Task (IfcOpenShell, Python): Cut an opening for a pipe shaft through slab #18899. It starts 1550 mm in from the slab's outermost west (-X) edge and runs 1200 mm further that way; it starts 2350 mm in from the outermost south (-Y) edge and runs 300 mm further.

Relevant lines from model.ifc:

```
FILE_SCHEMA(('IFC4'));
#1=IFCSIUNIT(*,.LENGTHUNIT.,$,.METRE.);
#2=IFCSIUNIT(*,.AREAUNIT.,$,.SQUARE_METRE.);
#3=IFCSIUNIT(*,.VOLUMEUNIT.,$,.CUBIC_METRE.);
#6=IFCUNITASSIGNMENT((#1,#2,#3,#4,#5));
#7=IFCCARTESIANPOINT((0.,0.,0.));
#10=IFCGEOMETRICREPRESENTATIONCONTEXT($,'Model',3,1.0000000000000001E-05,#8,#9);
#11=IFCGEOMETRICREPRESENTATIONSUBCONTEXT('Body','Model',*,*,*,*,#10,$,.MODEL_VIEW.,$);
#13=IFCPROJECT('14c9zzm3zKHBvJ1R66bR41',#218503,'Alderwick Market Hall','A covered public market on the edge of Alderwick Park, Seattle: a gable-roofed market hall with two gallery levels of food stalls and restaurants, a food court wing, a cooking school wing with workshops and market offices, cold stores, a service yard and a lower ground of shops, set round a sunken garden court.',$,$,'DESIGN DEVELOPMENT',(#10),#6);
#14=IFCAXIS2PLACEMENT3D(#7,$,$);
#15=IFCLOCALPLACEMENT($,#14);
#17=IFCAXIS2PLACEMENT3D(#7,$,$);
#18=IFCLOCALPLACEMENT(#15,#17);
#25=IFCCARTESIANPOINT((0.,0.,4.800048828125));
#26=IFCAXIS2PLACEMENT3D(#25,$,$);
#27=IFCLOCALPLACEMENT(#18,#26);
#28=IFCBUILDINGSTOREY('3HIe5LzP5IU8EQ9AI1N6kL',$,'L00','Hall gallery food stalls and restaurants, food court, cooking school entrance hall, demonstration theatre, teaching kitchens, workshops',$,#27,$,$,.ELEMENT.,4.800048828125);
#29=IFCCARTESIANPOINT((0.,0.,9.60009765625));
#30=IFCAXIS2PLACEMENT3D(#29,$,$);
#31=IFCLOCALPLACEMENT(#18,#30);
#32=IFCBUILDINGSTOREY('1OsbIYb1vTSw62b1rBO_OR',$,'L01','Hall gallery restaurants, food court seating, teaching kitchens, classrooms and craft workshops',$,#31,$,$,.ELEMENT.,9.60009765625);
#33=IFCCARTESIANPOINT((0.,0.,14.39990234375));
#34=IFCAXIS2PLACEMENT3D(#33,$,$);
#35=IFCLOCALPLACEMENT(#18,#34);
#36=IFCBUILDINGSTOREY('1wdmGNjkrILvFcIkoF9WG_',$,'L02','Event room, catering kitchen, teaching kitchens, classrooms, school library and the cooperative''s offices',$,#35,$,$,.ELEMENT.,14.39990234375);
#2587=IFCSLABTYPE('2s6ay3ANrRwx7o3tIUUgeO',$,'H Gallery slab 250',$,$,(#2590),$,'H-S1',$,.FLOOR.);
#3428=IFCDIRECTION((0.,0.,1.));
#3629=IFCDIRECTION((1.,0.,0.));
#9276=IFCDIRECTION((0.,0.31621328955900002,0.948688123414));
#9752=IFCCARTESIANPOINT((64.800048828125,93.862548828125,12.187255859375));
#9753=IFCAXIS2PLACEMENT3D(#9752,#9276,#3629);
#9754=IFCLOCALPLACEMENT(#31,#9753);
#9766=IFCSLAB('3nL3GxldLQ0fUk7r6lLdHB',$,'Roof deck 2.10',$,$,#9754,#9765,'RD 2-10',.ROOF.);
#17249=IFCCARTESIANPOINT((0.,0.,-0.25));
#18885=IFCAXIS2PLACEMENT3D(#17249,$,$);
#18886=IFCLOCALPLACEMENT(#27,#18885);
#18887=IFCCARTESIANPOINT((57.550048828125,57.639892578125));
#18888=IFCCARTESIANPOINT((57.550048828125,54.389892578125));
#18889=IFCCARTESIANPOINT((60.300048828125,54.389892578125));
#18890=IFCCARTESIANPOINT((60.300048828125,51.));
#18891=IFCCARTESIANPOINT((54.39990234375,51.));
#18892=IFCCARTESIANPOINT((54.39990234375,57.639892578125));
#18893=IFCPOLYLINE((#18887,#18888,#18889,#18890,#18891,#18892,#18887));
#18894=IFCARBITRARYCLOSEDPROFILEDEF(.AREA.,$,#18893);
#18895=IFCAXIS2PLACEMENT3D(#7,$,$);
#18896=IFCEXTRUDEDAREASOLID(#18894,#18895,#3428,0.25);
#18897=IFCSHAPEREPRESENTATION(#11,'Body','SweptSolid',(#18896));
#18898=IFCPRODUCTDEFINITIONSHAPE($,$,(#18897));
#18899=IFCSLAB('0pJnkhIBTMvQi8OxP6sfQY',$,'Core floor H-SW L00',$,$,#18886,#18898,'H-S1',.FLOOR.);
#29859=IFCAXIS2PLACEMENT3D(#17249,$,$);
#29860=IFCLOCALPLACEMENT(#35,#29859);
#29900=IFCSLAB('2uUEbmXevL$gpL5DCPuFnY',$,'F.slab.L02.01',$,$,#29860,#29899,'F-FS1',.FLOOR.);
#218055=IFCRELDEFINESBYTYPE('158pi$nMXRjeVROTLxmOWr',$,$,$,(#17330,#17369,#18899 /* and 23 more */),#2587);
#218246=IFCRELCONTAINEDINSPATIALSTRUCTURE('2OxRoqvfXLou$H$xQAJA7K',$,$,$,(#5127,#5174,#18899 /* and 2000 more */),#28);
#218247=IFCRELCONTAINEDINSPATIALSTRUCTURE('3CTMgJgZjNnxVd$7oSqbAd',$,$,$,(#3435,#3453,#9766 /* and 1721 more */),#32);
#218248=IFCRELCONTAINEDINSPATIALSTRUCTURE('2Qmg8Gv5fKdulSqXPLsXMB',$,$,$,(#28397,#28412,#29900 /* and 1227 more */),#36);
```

```python
import numpy as np
import ifcopenshell
import ifcopenshell.api.feature
import ifcopenshell.api.geometry
import ifcopenshell.api.root
import ifcopenshell.geom
import ifcopenshell.util.placement
import ifcopenshell.util.representation
import ifcopenshell.util.shape
import ifcopenshell.util.unit

model = ifcopenshell.open("model.ifc")
unit_scale = ifcopenshell.util.unit.calculate_unit_scale(model)
settings = ifcopenshell.geom.settings()


def volume(element):
    """Net volume in cubic metres, openings subtracted."""
    shape = ifcopenshell.geom.create_shape(settings, element)
    return ifcopenshell.util.shape.get_volume(shape.geometry)


slab = model.by_id(18899)
before = volume(slab)

# Extent in the slab's own axes, in metres. The edges named are its -X and -Y sides.
slab_shape = ifcopenshell.geom.create_shape(settings, slab)
vertices = ifcopenshell.util.shape.get_vertices(slab_shape.geometry)
x_min, y_min, bottom = vertices.min(axis=0)
top = vertices[:, 2].max()

opening = ifcopenshell.api.root.create_entity(model, ifc_class="IfcOpeningElement", name="Pipe shaft opening", predefined_type="OPENING")
context = ifcopenshell.util.representation.get_context(model, "Model", "Body", "MODEL_VIEW")
width, depth = 1.2, 0.3
outline = [(0.0, 0.0), (width, 0.0), (width, depth), (0.0, depth), (0.0, 0.0)]
# Overshoot both faces by 50 mm so the cut is clean.
shape = ifcopenshell.api.geometry.add_slab_representation(
    model, context=context, depth=top - bottom + 0.1, polyline=outline
)
ifcopenshell.api.geometry.assign_representation(model, product=opening, representation=shape)

matrix = ifcopenshell.util.placement.get_local_placement(slab.ObjectPlacement)
matrix[:, 3] = matrix @ np.append(np.array([x_min + 1.55, y_min + 2.35, bottom - 0.05]) / unit_scale, 1.0)
ifcopenshell.api.geometry.edit_object_placement(model, product=opening, matrix=matrix, is_si=False)
ifcopenshell.api.feature.add_feature(model, feature=opening, element=slab)

after = volume(slab)

print(f"slab volume {before:.3f} -> {after:.3f} m3")

model.write("model_rev.ifc")
```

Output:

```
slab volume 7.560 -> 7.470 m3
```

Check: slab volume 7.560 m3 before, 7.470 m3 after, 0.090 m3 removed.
